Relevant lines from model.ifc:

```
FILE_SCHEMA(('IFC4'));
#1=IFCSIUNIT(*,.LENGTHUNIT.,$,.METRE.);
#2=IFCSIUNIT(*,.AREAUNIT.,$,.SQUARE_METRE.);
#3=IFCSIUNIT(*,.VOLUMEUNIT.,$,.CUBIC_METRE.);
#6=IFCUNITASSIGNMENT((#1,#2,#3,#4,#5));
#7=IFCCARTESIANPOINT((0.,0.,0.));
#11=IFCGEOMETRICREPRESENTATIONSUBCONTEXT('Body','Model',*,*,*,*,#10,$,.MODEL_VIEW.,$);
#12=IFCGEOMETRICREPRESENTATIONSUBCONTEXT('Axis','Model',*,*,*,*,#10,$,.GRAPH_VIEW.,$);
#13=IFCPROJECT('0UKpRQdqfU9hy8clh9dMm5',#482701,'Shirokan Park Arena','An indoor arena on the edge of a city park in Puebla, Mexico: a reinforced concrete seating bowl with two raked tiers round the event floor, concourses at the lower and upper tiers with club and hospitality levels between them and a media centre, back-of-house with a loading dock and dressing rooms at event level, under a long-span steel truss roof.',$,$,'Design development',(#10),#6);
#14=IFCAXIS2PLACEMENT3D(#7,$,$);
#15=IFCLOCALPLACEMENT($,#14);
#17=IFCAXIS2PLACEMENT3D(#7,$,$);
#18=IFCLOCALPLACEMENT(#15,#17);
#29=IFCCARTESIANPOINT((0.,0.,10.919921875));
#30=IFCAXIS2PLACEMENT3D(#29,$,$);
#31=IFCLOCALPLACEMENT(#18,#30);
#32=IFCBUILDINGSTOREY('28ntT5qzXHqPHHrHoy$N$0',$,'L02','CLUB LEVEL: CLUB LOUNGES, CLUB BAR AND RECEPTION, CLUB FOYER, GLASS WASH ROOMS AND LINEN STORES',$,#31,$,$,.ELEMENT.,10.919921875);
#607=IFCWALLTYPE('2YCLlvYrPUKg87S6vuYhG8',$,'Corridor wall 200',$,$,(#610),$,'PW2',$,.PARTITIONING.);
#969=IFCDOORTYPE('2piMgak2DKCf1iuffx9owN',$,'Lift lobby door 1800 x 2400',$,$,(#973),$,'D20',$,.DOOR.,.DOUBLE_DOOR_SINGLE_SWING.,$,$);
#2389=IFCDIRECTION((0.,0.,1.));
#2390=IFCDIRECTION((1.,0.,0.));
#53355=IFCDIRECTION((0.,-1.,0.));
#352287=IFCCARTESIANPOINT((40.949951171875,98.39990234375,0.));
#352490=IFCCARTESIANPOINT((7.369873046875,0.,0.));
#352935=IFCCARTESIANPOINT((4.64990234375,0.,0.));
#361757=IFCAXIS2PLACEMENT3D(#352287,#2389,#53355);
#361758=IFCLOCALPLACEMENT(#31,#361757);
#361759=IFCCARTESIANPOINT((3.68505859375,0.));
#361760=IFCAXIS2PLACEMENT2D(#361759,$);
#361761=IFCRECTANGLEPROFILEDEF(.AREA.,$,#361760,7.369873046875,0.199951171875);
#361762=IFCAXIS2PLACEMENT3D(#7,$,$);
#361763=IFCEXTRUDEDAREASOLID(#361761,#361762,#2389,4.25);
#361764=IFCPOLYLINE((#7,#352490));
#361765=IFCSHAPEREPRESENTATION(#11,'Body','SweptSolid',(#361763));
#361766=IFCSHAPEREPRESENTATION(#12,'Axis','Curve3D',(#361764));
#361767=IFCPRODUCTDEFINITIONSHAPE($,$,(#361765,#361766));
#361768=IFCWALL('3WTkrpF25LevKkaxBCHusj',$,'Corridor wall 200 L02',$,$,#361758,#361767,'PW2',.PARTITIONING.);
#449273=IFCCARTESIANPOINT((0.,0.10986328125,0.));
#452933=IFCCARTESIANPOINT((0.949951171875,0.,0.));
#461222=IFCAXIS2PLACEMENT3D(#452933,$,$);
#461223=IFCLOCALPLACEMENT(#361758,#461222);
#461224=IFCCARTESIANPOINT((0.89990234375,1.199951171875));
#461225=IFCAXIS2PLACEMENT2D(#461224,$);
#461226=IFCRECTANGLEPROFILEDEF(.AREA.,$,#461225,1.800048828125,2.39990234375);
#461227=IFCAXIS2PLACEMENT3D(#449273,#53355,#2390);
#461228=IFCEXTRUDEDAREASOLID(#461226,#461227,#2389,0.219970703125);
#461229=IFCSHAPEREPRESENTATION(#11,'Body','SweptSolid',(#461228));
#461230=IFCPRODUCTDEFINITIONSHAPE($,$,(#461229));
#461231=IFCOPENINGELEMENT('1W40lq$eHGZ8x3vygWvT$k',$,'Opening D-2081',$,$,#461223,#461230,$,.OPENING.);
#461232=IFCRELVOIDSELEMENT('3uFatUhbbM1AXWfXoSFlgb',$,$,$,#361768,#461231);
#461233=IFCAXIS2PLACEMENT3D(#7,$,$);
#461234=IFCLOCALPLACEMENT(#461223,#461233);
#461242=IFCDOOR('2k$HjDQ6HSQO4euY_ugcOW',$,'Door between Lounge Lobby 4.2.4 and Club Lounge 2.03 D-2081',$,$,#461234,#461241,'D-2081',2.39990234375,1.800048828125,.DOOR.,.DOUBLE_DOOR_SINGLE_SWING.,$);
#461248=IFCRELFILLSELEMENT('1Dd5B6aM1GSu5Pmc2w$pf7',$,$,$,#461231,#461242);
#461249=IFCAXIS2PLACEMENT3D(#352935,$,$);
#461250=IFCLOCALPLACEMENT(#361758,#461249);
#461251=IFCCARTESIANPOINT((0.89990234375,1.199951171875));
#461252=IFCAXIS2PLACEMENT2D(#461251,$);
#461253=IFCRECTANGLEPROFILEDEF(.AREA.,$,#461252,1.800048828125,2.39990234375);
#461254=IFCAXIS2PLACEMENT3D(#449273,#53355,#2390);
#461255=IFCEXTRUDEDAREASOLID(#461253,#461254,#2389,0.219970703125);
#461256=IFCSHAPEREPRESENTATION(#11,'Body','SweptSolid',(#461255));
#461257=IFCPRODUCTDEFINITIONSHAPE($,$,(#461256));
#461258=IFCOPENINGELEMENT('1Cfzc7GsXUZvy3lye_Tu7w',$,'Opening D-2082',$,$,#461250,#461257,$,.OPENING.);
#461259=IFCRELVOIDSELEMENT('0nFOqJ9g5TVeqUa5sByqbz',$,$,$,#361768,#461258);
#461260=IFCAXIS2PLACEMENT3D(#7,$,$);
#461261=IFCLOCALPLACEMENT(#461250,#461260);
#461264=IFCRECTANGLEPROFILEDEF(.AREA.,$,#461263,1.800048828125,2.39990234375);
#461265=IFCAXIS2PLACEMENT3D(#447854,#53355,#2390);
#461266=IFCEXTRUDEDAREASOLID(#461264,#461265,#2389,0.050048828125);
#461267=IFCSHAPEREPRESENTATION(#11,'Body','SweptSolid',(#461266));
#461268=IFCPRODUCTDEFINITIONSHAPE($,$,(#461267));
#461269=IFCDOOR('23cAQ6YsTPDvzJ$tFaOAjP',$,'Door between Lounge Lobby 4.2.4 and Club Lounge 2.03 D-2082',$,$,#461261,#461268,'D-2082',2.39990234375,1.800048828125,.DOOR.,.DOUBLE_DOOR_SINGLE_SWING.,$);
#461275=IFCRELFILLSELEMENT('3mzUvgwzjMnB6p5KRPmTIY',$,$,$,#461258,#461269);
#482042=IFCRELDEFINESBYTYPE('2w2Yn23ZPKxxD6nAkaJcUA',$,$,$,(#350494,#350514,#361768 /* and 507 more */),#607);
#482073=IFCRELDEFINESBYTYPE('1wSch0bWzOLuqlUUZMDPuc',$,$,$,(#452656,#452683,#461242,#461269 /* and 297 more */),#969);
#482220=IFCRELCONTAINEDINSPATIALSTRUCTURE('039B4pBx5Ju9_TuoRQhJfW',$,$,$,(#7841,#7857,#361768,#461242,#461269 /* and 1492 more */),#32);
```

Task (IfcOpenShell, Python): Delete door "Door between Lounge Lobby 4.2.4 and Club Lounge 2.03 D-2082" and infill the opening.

```python
import ifcopenshell
import ifcopenshell.api.feature
import ifcopenshell.api.root
import ifcopenshell.geom
import ifcopenshell.util.shape

model = ifcopenshell.open("model.ifc")
settings = ifcopenshell.geom.settings()


def volume(element):
    """Net volume in cubic metres, openings subtracted."""
    shape = ifcopenshell.geom.create_shape(settings, element)
    return ifcopenshell.util.shape.get_volume(shape.geometry)


door = model.by_id(461269)
opening = door.FillsVoids[0].RelatingOpeningElement
wall = opening.VoidsElements[0].RelatingBuildingElement
before = volume(wall)

ifcopenshell.api.root.remove_product(model, product=door)
ifcopenshell.api.feature.remove_feature(model, feature=opening)

after = volume(wall)

print(f"wall volume {before:.3f} -> {after:.3f} m3")

model.write("model_updated.ifc")
```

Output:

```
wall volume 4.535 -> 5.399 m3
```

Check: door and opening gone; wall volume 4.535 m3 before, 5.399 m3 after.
